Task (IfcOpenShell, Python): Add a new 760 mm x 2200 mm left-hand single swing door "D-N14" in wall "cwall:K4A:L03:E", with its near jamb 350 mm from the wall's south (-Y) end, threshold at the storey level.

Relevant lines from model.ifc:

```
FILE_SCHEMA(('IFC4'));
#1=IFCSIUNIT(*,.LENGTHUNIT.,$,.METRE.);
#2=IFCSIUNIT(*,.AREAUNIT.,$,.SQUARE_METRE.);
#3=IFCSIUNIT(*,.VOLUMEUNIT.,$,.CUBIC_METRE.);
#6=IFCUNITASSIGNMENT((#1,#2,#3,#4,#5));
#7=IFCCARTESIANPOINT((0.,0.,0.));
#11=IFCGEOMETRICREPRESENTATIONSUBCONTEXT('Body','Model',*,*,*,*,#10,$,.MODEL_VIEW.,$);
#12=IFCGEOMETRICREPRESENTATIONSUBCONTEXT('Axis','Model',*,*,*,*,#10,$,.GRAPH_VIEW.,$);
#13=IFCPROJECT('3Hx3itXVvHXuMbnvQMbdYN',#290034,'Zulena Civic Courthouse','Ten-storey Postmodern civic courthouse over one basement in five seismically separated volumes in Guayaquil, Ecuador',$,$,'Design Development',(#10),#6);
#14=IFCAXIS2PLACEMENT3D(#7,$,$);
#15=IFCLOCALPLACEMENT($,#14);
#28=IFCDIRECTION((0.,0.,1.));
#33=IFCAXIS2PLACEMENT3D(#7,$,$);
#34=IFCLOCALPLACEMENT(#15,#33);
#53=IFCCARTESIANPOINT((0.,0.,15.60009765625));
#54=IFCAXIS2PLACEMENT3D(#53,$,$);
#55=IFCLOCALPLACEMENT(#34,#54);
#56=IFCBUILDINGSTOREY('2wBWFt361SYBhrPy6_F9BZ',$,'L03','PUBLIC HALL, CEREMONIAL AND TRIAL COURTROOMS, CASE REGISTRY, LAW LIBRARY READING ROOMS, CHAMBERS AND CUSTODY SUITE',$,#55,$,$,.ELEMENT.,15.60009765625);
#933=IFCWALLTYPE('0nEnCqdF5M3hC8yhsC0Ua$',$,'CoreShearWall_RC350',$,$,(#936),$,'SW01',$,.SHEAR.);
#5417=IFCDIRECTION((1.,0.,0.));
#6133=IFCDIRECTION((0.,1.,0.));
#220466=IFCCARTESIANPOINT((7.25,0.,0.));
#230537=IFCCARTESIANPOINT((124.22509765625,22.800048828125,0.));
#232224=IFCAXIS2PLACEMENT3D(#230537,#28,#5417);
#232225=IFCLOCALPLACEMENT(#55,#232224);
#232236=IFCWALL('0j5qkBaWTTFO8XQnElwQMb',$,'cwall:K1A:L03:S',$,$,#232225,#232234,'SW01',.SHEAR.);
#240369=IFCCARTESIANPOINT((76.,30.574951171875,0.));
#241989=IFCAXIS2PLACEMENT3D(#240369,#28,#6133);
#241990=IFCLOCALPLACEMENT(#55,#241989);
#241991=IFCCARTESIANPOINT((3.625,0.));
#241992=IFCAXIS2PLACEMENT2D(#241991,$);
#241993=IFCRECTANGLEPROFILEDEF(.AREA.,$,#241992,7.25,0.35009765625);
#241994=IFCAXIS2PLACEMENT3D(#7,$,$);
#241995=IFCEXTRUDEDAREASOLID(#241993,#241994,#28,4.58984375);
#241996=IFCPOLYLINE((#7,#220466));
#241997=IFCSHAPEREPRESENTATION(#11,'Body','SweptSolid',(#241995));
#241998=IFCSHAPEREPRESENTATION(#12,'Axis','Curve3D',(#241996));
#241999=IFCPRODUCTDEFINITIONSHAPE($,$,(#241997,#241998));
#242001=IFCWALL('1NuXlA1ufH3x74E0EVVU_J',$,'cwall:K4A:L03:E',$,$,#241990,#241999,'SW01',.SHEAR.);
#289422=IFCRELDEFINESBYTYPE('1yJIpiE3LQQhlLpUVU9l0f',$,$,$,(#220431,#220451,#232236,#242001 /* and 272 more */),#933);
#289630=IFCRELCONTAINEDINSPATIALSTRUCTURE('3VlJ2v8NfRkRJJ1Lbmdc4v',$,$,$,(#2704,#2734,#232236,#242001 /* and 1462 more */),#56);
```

```python
import numpy as np
import ifcopenshell
import ifcopenshell.api.feature
import ifcopenshell.api.geometry
import ifcopenshell.api.root
import ifcopenshell.api.spatial
import ifcopenshell.geom
import ifcopenshell.util.element
import ifcopenshell.util.placement
import ifcopenshell.util.representation
import ifcopenshell.util.shape
import ifcopenshell.util.unit

model = ifcopenshell.open("model.ifc")
unit_scale = ifcopenshell.util.unit.calculate_unit_scale(model)
settings = ifcopenshell.geom.settings()


def volume(element):
    """Net volume in cubic metres, openings subtracted."""
    shape = ifcopenshell.geom.create_shape(settings, element)
    return ifcopenshell.util.shape.get_volume(shape.geometry)


wall = model.by_guid("1NuXlA1ufH3x74E0EVVU_J")
storey = ifcopenshell.util.element.get_container(wall, ifc_class="IfcBuildingStorey")
context = ifcopenshell.util.representation.get_context(model, "Model", "Body", "MODEL_VIEW")
before = volume(wall)

width, height, from_end, sill = 0.76, 2.2, 0.35, 0.0  # metres

# The wall runs along its own X axis, and the end named is its -X end.
wall_shape = ifcopenshell.geom.create_shape(settings, wall)
x, y, z = ifcopenshell.util.shape.get_vertices(wall_shape.geometry).T
start = x.min() + from_end
face, thickness = float(y.min()), float(y.max() - y.min())
wall_matrix = ifcopenshell.util.placement.get_local_placement(wall.ObjectPlacement)
level = ifcopenshell.util.placement.get_local_placement(storey.ObjectPlacement)[2, 3]


def in_wall(x, y):
    """Placement at x, y metres in the wall's axes, at sill height."""
    matrix = wall_matrix.copy()
    matrix[:, 3] = wall_matrix @ np.array([x / unit_scale, y / unit_scale, 0.0, 1.0])
    matrix[2, 3] = level + sill / unit_scale
    return matrix


# Opening: a box that overshoots both wall faces by 50 mm.
opening = ifcopenshell.api.root.create_entity(model, ifc_class="IfcOpeningElement", predefined_type="OPENING")
box = ifcopenshell.api.geometry.add_wall_representation(
    model, context=context, length=width, height=height, thickness=thickness + 0.1
)
ifcopenshell.api.geometry.assign_representation(model, product=opening, representation=box)
ifcopenshell.api.geometry.edit_object_placement(model, product=opening, matrix=in_wall(start, face - 0.05), is_si=False)
ifcopenshell.api.feature.add_feature(model, feature=opening, element=wall)

door = ifcopenshell.api.root.create_entity(model, ifc_class="IfcDoor", name="D-N14", predefined_type="DOOR")
door.OverallWidth, door.OverallHeight = width / unit_scale, height / unit_scale
door.OperationType = "SINGLE_SWING_LEFT"
body = ifcopenshell.api.geometry.add_door_representation(
    model,
    context=context,
    overall_width=door.OverallWidth,
    overall_height=door.OverallHeight,
    operation_type="SINGLE_SWING_LEFT",
    lining_properties={"LiningDepth": thickness / unit_scale, "ThresholdDepth": thickness / unit_scale},
)
ifcopenshell.api.geometry.assign_representation(model, product=door, representation=body)
ifcopenshell.api.spatial.assign_container(model, products=[door], relating_structure=storey)
ifcopenshell.api.feature.add_filling(model, opening=opening, element=door)

# The lining spans the wall, so the door starts at the wall face.
ifcopenshell.api.geometry.edit_object_placement(model, product=door, matrix=in_wall(start, face), is_si=False)

after = volume(wall)

print(f"wall volume {before:.3f} -> {after:.3f} m3")

model.write("model_edited.ifc")
```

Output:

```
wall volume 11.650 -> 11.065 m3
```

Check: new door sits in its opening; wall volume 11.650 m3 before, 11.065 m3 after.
